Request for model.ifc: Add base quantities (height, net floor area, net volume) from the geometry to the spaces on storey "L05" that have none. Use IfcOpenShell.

First a look at what the model holds.

```python
import ifcopenshell
import ifcopenshell.util.element
import ifcopenshell.util.unit

model = ifcopenshell.open("model.ifc")
print(model.schema)
for unit_type in ("LENGTHUNIT", "AREAUNIT", "VOLUMEUNIT"):
    print(unit_type, ifcopenshell.util.unit.calculate_unit_scale(model, unit_type))
storey = next(s for s in model.by_type("IfcBuildingStorey") if s.Name == "L05")
spaces = [e for e in ifcopenshell.util.element.get_decomposition(storey) if e.is_a("IfcSpace")]
for e in sorted(spaces, key=lambda e: e.id()):
    print(e.id(), e.is_a(), e.Name, list(ifcopenshell.util.element.get_psets(e, qtos_only=True)), sep=" | ")
```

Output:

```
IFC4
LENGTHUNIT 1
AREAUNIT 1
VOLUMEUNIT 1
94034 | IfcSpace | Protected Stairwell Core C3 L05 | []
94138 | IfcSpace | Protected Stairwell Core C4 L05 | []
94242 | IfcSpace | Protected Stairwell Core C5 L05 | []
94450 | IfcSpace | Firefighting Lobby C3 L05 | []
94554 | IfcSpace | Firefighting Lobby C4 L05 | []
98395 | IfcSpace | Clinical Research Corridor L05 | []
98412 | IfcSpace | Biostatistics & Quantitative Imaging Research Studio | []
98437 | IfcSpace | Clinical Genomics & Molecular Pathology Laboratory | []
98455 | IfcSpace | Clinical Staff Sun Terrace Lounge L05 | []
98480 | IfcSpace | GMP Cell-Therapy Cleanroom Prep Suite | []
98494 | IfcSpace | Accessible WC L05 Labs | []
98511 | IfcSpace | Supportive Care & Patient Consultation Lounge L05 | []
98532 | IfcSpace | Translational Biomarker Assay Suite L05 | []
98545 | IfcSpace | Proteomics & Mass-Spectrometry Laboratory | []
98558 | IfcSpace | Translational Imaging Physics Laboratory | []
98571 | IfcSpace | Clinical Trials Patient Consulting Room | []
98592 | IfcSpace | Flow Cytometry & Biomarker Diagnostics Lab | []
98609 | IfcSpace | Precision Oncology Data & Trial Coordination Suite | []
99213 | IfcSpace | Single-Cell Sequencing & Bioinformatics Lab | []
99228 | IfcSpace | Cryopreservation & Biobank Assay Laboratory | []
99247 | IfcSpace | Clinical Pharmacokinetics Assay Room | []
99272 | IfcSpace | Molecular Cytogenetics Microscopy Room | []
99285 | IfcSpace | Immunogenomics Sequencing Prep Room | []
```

```python
import ifcopenshell
import ifcopenshell.api.pset
import ifcopenshell.geom
import ifcopenshell.util.element
import ifcopenshell.util.shape
import ifcopenshell.util.unit

model = ifcopenshell.open("model.ifc")
unit_scale = ifcopenshell.util.unit.calculate_unit_scale(model)
area_scale = ifcopenshell.util.unit.calculate_unit_scale(model, "AREAUNIT")
volume_scale = ifcopenshell.util.unit.calculate_unit_scale(model, "VOLUMEUNIT")
settings = ifcopenshell.geom.settings()

storey = next(s for s in model.by_type("IfcBuildingStorey") if s.Name == "L05")
spaces = [e for e in ifcopenshell.util.element.get_decomposition(storey) if e.is_a("IfcSpace")]

for e in sorted(spaces, key=lambda e: e.id()):
    if ifcopenshell.util.element.get_psets(e, qtos_only=True, should_inherit=False):
        continue
    # Geometry comes back in metres, in the element's own axes.
    shape = ifcopenshell.geom.create_shape(settings, e)
    values = {
        "Height": ifcopenshell.util.shape.get_z(shape.geometry) / unit_scale,
        "NetFloorArea": ifcopenshell.util.shape.get_footprint_area(shape.geometry) / area_scale,
        "NetVolume": ifcopenshell.util.shape.get_volume(shape.geometry) / volume_scale,
    }
    qto = ifcopenshell.api.pset.add_qto(model, product=e, name="Qto_SpaceBaseQuantities")
    ifcopenshell.api.pset.edit_qto(model, qto=qto, properties=values)
    print(e.id(), {k: round(v, 3) for k, v in values.items()})

model.write("model_v2.ifc")
```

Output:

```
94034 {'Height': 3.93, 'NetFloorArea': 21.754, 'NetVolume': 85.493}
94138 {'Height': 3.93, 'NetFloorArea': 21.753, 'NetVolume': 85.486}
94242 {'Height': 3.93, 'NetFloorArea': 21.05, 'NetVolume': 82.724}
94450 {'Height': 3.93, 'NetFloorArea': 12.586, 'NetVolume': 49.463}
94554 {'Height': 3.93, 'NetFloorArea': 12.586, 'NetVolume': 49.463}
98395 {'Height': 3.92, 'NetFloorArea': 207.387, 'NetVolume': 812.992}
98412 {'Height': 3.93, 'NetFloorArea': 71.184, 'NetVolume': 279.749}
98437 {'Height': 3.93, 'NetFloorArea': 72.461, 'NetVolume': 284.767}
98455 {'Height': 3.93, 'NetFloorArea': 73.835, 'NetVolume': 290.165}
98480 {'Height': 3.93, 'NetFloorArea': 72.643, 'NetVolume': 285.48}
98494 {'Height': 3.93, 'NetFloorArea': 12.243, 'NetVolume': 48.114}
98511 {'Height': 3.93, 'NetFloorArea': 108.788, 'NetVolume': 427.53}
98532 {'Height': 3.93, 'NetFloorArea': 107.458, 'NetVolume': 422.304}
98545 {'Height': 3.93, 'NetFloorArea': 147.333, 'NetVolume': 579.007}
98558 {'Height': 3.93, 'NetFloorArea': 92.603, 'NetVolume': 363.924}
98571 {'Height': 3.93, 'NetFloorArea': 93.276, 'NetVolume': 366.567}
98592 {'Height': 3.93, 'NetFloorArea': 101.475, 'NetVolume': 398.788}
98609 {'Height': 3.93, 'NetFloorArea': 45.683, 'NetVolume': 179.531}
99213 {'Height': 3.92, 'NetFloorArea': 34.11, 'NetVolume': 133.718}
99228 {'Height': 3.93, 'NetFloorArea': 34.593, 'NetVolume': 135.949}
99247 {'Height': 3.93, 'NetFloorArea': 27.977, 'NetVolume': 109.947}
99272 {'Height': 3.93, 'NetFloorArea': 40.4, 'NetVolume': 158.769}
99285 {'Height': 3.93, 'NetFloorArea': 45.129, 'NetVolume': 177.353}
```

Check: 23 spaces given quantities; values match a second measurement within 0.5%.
